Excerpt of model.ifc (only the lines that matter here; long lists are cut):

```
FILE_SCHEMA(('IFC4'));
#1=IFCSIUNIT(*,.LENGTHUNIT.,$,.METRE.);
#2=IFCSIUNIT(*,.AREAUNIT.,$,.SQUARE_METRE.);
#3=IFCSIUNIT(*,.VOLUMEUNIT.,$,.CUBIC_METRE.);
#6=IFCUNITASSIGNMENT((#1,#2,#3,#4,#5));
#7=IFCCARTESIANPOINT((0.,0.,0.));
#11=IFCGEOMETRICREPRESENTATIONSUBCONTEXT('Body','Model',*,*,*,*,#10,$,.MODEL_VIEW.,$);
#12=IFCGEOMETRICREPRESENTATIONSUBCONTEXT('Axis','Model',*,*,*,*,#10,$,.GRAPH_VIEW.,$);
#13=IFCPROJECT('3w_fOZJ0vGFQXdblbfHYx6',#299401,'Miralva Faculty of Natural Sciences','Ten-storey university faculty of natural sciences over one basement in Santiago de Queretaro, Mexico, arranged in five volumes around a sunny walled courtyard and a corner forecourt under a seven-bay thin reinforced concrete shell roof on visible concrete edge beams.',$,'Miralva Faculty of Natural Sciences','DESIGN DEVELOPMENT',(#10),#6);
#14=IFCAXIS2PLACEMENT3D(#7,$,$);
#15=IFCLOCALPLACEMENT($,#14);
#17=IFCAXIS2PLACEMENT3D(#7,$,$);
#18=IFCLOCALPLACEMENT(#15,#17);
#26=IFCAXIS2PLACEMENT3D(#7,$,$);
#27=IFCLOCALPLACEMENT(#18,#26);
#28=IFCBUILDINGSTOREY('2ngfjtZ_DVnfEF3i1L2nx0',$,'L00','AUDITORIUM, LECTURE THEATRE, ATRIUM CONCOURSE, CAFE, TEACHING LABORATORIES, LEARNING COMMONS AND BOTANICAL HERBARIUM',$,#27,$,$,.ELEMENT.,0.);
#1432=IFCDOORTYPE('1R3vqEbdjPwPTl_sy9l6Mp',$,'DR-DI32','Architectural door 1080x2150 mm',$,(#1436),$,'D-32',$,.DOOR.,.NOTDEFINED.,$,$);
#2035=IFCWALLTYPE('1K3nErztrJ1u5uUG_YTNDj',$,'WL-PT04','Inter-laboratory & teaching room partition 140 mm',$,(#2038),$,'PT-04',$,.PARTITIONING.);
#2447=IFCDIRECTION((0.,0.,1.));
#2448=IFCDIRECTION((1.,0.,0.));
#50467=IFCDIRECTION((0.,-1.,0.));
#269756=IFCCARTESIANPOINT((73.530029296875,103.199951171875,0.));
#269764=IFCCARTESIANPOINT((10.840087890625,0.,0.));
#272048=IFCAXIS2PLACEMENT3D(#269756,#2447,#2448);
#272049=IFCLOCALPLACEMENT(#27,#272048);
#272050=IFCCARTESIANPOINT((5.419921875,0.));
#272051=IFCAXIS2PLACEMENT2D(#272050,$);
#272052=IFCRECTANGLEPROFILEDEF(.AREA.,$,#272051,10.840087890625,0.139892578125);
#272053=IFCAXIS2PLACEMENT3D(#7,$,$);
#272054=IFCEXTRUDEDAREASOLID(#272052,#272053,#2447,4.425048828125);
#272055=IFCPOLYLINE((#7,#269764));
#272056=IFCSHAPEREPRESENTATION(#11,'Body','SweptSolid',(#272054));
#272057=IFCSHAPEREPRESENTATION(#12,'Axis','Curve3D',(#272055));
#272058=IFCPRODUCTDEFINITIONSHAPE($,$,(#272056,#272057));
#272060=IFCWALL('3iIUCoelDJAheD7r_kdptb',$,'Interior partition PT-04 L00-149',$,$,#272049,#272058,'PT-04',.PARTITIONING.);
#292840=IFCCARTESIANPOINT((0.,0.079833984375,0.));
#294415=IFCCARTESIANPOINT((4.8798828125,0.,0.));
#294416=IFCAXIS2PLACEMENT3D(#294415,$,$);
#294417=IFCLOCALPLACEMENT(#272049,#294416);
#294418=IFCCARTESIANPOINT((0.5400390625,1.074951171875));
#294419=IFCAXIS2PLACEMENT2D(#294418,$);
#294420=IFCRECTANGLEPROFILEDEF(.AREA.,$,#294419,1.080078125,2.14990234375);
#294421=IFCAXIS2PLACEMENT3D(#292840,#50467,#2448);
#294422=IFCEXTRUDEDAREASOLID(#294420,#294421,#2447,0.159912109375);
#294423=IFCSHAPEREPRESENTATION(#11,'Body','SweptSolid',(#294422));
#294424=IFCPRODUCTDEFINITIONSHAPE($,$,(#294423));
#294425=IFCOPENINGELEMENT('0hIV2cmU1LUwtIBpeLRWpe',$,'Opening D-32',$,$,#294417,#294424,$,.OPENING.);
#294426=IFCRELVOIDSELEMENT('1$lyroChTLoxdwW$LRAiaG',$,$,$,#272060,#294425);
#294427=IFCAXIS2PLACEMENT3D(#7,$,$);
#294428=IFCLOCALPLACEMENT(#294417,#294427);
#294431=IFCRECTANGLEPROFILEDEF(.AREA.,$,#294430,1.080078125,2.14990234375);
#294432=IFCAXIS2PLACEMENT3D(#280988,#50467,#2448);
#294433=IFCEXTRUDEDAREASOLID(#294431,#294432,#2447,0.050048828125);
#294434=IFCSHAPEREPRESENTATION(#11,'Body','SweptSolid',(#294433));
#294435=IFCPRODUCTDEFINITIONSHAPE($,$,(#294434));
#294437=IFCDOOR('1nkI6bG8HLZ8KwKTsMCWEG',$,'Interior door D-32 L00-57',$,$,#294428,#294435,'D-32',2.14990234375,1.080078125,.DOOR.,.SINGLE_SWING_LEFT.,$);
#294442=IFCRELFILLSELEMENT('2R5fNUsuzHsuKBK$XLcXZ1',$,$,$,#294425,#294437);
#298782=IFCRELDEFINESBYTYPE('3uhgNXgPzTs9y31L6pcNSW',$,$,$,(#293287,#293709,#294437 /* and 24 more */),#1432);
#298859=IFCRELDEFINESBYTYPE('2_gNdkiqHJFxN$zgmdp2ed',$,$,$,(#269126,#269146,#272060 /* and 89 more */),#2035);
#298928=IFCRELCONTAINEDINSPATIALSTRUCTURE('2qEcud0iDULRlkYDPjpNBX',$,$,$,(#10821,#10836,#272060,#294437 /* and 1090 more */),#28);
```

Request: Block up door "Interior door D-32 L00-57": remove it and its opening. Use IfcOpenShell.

```python
import ifcopenshell
import ifcopenshell.api.feature
import ifcopenshell.api.root
import ifcopenshell.geom
import ifcopenshell.util.shape

model = ifcopenshell.open("model.ifc")
settings = ifcopenshell.geom.settings()


def volume(element):
    """Net volume in cubic metres, openings subtracted."""
    shape = ifcopenshell.geom.create_shape(settings, element)
    return ifcopenshell.util.shape.get_volume(shape.geometry)


door = model.by_guid("1nkI6bG8HLZ8KwKTsMCWEG")
opening = door.FillsVoids[0].RelatingOpeningElement
wall = opening.VoidsElements[0].RelatingBuildingElement
before = volume(wall)

ifcopenshell.api.root.remove_product(model, product=door)
ifcopenshell.api.feature.remove_feature(model, feature=opening)

after = volume(wall)

print(f"wall volume {before:.3f} -> {after:.3f} m3")

model.write("model_rev.ifc")
```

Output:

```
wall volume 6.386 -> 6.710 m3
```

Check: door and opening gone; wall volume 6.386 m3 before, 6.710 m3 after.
